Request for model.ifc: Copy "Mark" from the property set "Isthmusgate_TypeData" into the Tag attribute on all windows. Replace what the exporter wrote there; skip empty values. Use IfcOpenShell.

First a look at what the model holds.

```python
import ifcopenshell
import ifcopenshell.util.element

model = ifcopenshell.open("model.ifc")
print(model.schema)
windows = model.by_type("IfcWindow")
print(len(windows), "windows")
for e in windows[:8]:
    source = ifcopenshell.util.element.get_pset(e, "Isthmusgate_TypeData", "Mark")
    target = e.Tag
    print(e.id(), repr(source), repr(target), sep=" | ")
```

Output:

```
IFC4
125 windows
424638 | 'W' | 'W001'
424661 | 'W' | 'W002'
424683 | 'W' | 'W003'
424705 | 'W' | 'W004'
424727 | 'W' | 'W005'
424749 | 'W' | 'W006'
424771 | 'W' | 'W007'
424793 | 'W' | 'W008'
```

```python
import ifcopenshell
import ifcopenshell.util.element

model = ifcopenshell.open("model.ifc")

count = 0
for e in model.by_type("IfcWindow"):
    value = ifcopenshell.util.element.get_pset(e, "Isthmusgate_TypeData", "Mark")
    current = e.Tag
    if not value or not value.strip() or current == value:
        continue
    e.Tag = value
    count += 1

print(count, "windows updated")

model.write("model-out.ifc")
```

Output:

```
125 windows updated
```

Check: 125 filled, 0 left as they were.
